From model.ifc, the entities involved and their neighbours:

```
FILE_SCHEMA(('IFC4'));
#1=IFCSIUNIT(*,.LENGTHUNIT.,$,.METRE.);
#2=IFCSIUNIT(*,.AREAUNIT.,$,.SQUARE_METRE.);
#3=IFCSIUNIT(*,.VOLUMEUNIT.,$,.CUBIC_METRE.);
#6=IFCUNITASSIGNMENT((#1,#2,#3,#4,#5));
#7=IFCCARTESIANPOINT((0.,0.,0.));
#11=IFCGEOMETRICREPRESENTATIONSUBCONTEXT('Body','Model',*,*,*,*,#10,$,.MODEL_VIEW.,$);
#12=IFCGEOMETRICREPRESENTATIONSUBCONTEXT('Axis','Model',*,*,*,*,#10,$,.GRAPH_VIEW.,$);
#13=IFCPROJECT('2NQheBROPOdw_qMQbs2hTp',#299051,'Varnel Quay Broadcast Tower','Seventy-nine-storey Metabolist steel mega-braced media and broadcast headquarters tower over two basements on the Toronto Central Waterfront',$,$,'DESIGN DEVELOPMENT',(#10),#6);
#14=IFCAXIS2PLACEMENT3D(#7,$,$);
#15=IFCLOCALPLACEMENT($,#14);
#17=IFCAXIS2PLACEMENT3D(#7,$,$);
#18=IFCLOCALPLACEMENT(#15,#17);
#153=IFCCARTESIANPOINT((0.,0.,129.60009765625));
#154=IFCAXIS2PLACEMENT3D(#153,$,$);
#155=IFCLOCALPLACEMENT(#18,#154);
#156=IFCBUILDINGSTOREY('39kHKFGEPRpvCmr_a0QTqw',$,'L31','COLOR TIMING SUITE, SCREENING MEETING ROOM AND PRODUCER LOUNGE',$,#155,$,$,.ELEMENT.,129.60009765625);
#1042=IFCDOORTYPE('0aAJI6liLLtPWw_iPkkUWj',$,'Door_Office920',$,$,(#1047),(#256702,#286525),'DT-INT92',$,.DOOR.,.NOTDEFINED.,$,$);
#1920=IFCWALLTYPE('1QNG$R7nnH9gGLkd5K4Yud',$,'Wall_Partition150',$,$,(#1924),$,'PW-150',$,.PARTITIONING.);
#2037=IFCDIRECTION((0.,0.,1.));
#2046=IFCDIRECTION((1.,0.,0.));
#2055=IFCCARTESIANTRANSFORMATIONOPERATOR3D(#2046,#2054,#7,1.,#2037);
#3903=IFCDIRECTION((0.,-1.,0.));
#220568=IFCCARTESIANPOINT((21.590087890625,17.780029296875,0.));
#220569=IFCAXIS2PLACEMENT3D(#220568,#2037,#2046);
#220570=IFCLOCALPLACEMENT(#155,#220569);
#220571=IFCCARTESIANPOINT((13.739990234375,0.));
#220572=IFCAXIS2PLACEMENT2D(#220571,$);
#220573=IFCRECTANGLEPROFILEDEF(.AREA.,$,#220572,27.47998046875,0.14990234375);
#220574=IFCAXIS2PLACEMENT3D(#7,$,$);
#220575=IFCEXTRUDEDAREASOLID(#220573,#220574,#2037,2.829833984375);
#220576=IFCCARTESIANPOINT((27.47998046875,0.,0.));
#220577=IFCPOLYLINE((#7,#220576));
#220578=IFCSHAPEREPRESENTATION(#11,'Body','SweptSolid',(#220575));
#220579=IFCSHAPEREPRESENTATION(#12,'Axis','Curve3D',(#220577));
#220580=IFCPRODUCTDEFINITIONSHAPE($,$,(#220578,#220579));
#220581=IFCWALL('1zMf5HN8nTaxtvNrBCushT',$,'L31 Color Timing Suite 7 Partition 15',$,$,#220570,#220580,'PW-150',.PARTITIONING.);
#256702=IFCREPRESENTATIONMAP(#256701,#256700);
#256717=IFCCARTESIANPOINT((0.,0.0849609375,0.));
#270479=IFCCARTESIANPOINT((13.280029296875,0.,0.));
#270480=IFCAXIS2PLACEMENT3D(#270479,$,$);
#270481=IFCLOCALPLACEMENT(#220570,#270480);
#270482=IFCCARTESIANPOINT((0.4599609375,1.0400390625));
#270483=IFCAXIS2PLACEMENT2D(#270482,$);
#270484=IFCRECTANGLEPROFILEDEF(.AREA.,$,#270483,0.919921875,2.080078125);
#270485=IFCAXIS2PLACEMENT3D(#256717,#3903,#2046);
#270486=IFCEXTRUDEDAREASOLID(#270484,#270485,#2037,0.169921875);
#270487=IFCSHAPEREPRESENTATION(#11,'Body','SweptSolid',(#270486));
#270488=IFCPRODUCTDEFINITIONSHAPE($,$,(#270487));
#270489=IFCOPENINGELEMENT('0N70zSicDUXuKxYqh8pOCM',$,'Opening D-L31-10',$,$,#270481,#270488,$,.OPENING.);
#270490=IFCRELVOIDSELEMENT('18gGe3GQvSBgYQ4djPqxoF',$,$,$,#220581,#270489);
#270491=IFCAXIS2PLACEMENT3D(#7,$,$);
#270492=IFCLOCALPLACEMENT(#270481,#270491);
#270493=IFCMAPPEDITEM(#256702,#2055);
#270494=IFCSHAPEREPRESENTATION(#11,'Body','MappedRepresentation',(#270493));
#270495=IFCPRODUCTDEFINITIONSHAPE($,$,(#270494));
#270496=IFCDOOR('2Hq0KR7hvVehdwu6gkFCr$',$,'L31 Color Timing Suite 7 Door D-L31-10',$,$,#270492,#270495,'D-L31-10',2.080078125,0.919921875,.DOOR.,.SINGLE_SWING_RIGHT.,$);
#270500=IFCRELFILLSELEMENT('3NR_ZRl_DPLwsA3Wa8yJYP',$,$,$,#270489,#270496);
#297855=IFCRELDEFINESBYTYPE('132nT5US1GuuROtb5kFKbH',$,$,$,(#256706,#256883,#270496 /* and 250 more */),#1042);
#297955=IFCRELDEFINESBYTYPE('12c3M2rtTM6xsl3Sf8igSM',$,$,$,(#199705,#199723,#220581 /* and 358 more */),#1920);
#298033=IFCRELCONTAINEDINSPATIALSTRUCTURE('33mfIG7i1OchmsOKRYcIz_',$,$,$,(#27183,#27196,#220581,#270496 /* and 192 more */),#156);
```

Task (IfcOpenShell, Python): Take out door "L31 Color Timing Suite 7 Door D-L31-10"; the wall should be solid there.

```python
import ifcopenshell
import ifcopenshell.api.feature
import ifcopenshell.api.root
import ifcopenshell.geom
import ifcopenshell.util.shape

model = ifcopenshell.open("model.ifc")
settings = ifcopenshell.geom.settings()


def volume(element):
    """Net volume in cubic metres, openings subtracted."""
    shape = ifcopenshell.geom.create_shape(settings, element)
    return ifcopenshell.util.shape.get_volume(shape.geometry)


door = model.by_guid("2Hq0KR7hvVehdwu6gkFCr$")
opening = door.FillsVoids[0].RelatingOpeningElement
wall = opening.VoidsElements[0].RelatingBuildingElement
before = volume(wall)

ifcopenshell.api.root.remove_product(model, product=door)
ifcopenshell.api.feature.remove_feature(model, feature=opening)

after = volume(wall)

print(f"wall volume {before:.3f} -> {after:.3f} m3")

model.write("model_v2.ifc")
```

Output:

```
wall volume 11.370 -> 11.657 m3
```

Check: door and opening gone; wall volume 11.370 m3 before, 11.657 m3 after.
